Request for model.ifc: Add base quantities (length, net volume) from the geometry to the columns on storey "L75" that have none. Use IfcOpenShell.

First a look at what the model holds.

```python
import ifcopenshell
import ifcopenshell.util.element
import ifcopenshell.util.unit

model = ifcopenshell.open("model.ifc")
print(model.schema)
for unit_type in ("LENGTHUNIT", "AREAUNIT", "VOLUMEUNIT"):
    print(unit_type, ifcopenshell.util.unit.calculate_unit_scale(model, unit_type))
storey = next(s for s in model.by_type("IfcBuildingStorey") if s.Name == "L75")
columns = [e for e in ifcopenshell.util.element.get_decomposition(storey) if e.is_a("IfcColumn")]
for e in sorted(columns, key=lambda e: e.id()):
    print(e.id(), e.is_a(), e.Name, list(ifcopenshell.util.element.get_psets(e, qtos_only=True)), sep=" | ")
```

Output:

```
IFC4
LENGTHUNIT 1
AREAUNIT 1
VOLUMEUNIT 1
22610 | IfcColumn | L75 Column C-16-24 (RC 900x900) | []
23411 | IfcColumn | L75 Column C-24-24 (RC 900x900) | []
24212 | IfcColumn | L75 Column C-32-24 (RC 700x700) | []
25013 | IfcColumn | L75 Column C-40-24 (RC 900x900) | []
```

```python
import ifcopenshell
import ifcopenshell.api.pset
import ifcopenshell.geom
import ifcopenshell.util.element
import ifcopenshell.util.shape
import ifcopenshell.util.unit

model = ifcopenshell.open("model.ifc")
unit_scale = ifcopenshell.util.unit.calculate_unit_scale(model)
volume_scale = ifcopenshell.util.unit.calculate_unit_scale(model, "VOLUMEUNIT")
settings = ifcopenshell.geom.settings()

storey = next(s for s in model.by_type("IfcBuildingStorey") if s.Name == "L75")
columns = [e for e in ifcopenshell.util.element.get_decomposition(storey) if e.is_a("IfcColumn")]

for e in sorted(columns, key=lambda e: e.id()):
    if ifcopenshell.util.element.get_psets(e, qtos_only=True, should_inherit=False):
        continue
    # Geometry comes back in metres, in the element's own axes.
    shape = ifcopenshell.geom.create_shape(settings, e)
    values = {
        "Length": ifcopenshell.util.shape.get_z(shape.geometry) / unit_scale,
        "NetVolume": ifcopenshell.util.shape.get_volume(shape.geometry) / volume_scale,
    }
    qto = ifcopenshell.api.pset.add_qto(model, product=e, name="Qto_ColumnBaseQuantities")
    ifcopenshell.api.pset.edit_qto(model, qto=qto, properties=values)
    print(e.id(), {k: round(v, 3) for k, v in values.items()})

model.write("model_rev.ifc")
```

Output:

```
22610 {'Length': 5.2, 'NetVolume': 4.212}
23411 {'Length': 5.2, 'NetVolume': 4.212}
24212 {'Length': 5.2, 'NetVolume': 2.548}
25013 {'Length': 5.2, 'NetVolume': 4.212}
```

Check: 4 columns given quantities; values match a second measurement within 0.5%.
